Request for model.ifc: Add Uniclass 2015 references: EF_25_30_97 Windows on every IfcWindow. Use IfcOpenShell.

First a look at what the model holds.

```python
import ifcopenshell

model = ifcopenshell.open("model.ifc")
print(model.schema)
print("classifications:", [c.Name for c in model.by_type("IfcClassification")])
for ifc_class in ("IfcDoor", "IfcRoof", "IfcStair", "IfcWall", "IfcWindow"):
    print(ifc_class, len(model.by_type(ifc_class)))
```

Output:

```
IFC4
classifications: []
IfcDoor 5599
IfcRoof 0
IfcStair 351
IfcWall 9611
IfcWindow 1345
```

```python
import ifcopenshell
import ifcopenshell.api.classification

model = ifcopenshell.open("model.ifc")

system = ifcopenshell.api.classification.add_classification(model, classification="Uniclass 2015")

codes = {
    "IfcWindow": ("EF_25_30_97", "Windows"),
}
for ifc_class, (code, name) in codes.items():
    products = model.by_type(ifc_class)
    ifcopenshell.api.classification.add_reference(
        model, products=products, classification=system, identification=code, name=name
    )
    print(code, len(products))

model.write("model_edited.ifc")
```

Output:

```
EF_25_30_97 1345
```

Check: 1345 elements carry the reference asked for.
